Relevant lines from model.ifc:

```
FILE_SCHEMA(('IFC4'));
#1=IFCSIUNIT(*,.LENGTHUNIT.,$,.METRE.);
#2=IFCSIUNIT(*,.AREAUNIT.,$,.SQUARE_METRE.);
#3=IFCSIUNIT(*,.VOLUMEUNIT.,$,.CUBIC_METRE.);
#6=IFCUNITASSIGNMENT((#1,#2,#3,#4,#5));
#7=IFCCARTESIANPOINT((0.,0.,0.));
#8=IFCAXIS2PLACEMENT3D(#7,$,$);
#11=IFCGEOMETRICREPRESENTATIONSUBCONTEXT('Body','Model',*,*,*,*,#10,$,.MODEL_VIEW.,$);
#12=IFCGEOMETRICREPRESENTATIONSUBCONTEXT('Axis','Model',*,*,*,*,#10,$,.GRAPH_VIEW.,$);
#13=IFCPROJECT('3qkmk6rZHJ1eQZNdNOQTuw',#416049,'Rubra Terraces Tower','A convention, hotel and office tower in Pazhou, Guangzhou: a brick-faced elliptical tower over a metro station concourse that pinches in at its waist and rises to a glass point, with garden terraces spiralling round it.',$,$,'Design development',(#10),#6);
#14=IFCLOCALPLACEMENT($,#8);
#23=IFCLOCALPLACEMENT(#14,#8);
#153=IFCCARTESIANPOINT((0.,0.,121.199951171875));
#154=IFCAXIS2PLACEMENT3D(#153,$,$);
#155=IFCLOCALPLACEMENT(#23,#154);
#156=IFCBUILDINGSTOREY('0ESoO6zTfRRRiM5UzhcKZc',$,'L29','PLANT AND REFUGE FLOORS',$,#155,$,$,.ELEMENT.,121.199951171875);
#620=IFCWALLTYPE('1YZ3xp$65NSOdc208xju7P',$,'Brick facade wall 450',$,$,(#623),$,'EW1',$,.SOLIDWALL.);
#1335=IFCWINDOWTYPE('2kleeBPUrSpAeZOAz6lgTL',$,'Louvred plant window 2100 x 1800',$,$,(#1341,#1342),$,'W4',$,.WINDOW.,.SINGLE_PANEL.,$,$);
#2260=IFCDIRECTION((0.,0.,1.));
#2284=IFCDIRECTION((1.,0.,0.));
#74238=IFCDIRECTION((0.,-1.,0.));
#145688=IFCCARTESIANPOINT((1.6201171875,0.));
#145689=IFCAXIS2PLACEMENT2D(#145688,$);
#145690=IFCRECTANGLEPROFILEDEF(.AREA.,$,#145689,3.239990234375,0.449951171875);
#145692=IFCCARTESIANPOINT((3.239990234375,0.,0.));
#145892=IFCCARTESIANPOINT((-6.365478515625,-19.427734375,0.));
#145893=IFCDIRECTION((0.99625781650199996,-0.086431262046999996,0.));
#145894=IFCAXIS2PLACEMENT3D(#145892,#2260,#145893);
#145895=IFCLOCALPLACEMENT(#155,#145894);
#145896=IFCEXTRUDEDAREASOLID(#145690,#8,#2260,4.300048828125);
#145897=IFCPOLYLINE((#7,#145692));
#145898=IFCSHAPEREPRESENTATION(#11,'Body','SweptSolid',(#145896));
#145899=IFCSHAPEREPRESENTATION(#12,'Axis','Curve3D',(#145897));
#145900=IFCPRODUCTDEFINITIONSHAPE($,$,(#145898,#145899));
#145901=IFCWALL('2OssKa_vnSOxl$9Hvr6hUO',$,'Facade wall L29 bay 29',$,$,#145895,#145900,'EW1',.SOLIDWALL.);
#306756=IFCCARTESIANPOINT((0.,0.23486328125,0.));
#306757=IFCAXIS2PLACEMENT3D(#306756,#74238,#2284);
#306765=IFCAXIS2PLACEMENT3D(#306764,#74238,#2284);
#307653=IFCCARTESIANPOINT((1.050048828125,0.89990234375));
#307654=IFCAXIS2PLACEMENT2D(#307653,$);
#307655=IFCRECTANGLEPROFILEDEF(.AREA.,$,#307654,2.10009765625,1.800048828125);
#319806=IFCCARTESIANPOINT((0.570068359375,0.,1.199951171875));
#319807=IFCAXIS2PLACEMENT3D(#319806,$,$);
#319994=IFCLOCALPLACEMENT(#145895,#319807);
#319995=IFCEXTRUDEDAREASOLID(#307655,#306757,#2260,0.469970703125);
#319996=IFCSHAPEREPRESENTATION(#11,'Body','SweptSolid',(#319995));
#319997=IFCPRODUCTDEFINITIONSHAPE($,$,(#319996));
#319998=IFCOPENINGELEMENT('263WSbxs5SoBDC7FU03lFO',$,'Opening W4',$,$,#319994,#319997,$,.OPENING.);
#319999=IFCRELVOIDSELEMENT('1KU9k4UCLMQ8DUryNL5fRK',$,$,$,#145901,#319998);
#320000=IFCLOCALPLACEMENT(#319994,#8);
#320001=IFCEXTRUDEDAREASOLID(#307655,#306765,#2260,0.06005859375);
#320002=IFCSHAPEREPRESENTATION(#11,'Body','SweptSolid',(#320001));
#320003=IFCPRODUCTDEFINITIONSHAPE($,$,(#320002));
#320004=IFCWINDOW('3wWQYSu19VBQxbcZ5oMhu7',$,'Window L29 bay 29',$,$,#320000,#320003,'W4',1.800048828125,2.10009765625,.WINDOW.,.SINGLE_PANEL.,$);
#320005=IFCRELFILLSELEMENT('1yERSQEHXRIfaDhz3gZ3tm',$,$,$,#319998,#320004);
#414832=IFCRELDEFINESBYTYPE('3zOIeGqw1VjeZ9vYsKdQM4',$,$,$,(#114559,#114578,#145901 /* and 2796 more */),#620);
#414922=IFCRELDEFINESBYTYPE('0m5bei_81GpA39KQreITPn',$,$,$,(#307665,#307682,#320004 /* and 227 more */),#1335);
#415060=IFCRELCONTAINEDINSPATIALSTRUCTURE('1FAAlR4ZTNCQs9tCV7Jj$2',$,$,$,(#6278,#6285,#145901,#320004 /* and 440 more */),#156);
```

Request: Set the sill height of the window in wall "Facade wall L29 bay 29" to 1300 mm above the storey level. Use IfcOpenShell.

```python
import numpy as np
import ifcopenshell
import ifcopenshell.api.geometry
import ifcopenshell.geom
import ifcopenshell.util.element
import ifcopenshell.util.placement
import ifcopenshell.util.shape
import ifcopenshell.util.unit

model = ifcopenshell.open("model.ifc")
unit_scale = ifcopenshell.util.unit.calculate_unit_scale(model)

window = model.by_guid("3wWQYSu19VBQxbcZ5oMhu7")
opening = window.FillsVoids[0].RelatingOpeningElement
storey = ifcopenshell.util.element.get_container(window, ifc_class="IfcBuildingStorey")
level = ifcopenshell.util.placement.get_local_placement(storey.ObjectPlacement)[2, 3]

# The opening's origin need not be at the sill, so measure its lowest point.
shape = ifcopenshell.geom.create_shape(ifcopenshell.geom.settings(), opening)
bottom = ifcopenshell.util.shape.get_shape_bottom_elevation(shape, shape.geometry) / unit_scale
dz = level + 1.3 - bottom

shift = np.array([0.0, 0.0, dz])
# The window is placed relative to its opening, so it follows when the opening moves.
matrix = ifcopenshell.util.placement.get_local_placement(opening.ObjectPlacement)
matrix[:3, 3] += shift
ifcopenshell.api.geometry.edit_object_placement(
    model, product=opening, matrix=matrix, is_si=False, should_transform_children=True
)

print(f"moved by {dz * unit_scale:+.3f} m")

model.write("model_updated.ifc")
```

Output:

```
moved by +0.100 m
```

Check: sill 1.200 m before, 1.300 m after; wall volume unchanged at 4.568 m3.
